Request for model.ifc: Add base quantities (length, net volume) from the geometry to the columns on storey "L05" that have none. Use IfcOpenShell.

First a look at what the model holds.

```python
import ifcopenshell
import ifcopenshell.util.element
import ifcopenshell.util.unit

model = ifcopenshell.open("model.ifc")
print(model.schema)
for unit_type in ("LENGTHUNIT", "AREAUNIT", "VOLUMEUNIT"):
    print(unit_type, ifcopenshell.util.unit.calculate_unit_scale(model, unit_type))
storey = next(s for s in model.by_type("IfcBuildingStorey") if s.Name == "L05")
columns = [e for e in ifcopenshell.util.element.get_decomposition(storey) if e.is_a("IfcColumn")]
for e in sorted(columns, key=lambda e: e.id()):
    print(e.id(), e.is_a(), e.Name, list(ifcopenshell.util.element.get_psets(e, qtos_only=True)), sep=" | ")
```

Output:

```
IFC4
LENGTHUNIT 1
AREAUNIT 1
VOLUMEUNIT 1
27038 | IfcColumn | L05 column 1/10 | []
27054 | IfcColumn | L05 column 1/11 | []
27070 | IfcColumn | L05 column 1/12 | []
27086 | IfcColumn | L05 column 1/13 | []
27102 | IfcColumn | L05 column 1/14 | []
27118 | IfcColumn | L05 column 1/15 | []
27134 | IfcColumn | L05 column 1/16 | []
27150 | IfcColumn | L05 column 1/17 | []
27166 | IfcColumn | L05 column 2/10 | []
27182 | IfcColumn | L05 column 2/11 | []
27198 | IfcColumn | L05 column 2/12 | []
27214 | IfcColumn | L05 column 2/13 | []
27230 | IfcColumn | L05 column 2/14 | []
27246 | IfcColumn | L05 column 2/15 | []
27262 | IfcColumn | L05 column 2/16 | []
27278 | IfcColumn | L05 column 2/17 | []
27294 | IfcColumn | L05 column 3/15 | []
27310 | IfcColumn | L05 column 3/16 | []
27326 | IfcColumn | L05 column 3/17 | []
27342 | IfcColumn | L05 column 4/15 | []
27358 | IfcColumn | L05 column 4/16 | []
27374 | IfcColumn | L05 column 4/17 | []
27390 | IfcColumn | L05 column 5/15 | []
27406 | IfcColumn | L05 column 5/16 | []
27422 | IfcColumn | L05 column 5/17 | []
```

```python
import ifcopenshell
import ifcopenshell.api.pset
import ifcopenshell.geom
import ifcopenshell.util.element
import ifcopenshell.util.shape
import ifcopenshell.util.unit

model = ifcopenshell.open("model.ifc")
unit_scale = ifcopenshell.util.unit.calculate_unit_scale(model)
volume_scale = ifcopenshell.util.unit.calculate_unit_scale(model, "VOLUMEUNIT")
settings = ifcopenshell.geom.settings()

storey = next(s for s in model.by_type("IfcBuildingStorey") if s.Name == "L05")
columns = [e for e in ifcopenshell.util.element.get_decomposition(storey) if e.is_a("IfcColumn")]

for e in sorted(columns, key=lambda e: e.id()):
    if ifcopenshell.util.element.get_psets(e, qtos_only=True, should_inherit=False):
        continue
    # Geometry comes back in metres, in the element's own axes.
    shape = ifcopenshell.geom.create_shape(settings, e)
    values = {
        "Length": ifcopenshell.util.shape.get_z(shape.geometry) / unit_scale,
        "NetVolume": ifcopenshell.util.shape.get_volume(shape.geometry) / volume_scale,
    }
    qto = ifcopenshell.api.pset.add_qto(model, product=e, name="Qto_ColumnBaseQuantities")
    ifcopenshell.api.pset.edit_qto(model, qto=qto, properties=values)
    print(e.id(), {k: round(v, 3) for k, v in values.items()})

model.write("model_v2.ifc")
```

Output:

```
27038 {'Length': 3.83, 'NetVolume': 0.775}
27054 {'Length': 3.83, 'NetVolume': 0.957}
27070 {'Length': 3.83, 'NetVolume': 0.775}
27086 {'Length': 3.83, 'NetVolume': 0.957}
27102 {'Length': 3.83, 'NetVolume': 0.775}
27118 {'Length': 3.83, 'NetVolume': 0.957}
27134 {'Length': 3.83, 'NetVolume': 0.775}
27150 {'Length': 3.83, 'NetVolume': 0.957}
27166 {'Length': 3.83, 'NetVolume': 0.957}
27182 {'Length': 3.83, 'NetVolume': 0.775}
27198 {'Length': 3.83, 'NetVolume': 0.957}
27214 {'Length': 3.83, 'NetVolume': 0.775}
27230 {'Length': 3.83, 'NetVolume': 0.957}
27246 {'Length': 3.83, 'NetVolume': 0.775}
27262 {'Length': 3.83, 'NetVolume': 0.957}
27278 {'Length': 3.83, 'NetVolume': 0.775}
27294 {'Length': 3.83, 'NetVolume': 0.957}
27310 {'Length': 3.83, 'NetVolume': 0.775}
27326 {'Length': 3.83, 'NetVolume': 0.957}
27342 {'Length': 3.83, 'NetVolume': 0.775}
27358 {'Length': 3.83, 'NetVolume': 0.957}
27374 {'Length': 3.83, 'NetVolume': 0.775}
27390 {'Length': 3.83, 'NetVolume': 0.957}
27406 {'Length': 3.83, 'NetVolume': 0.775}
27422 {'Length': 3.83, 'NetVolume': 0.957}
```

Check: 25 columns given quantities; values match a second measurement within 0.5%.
